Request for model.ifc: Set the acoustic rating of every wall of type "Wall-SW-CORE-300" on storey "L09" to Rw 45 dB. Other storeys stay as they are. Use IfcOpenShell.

First a look at what the model holds.

```python
import ifcopenshell
import ifcopenshell.util.element

model = ifcopenshell.open("model.ifc")
print(model.schema)
storey = next(s for s in model.by_type("IfcBuildingStorey") if s.Name == "L09")
walls = [e for e in ifcopenshell.util.element.get_decomposition(storey) if e.is_a("IfcWall")]
seen = {}
for e in walls:
    element_type = ifcopenshell.util.element.get_type(e)
    key = (element_type.Name if element_type != e and element_type else None, ifcopenshell.util.element.get_pset(e, "Pset_WallCommon", "AcousticRating"))
    seen[key] = seen.get(key, 0) + 1
for (name, value), count in sorted(seen.items(), key=str):
    print(count, "x", name, "|", value)
```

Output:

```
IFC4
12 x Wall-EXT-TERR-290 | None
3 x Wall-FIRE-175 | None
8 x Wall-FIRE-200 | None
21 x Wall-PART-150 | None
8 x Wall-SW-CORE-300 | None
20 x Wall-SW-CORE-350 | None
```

```python
import ifcopenshell
import ifcopenshell.api.pset
import ifcopenshell.util.element

model = ifcopenshell.open("model.ifc")

storey = next(s for s in model.by_type("IfcBuildingStorey") if s.Name == "L09")
walls = [e for e in ifcopenshell.util.element.get_decomposition(storey) if e.is_a("IfcWall")]

count = 0
for e in walls:
    element_type = ifcopenshell.util.element.get_type(e)
    if element_type in (None, e) or element_type.Name != "Wall-SW-CORE-300":
        continue
    # add_pset returns the element's existing set when there is one.
    pset = ifcopenshell.api.pset.add_pset(model, product=e, name="Pset_WallCommon")
    ifcopenshell.api.pset.edit_pset(model, pset=pset, properties={"AcousticRating": "Rw 45 dB"})
    count += 1

print(count, "walls updated")

model.write("model-out.ifc")
```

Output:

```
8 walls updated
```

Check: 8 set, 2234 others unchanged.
